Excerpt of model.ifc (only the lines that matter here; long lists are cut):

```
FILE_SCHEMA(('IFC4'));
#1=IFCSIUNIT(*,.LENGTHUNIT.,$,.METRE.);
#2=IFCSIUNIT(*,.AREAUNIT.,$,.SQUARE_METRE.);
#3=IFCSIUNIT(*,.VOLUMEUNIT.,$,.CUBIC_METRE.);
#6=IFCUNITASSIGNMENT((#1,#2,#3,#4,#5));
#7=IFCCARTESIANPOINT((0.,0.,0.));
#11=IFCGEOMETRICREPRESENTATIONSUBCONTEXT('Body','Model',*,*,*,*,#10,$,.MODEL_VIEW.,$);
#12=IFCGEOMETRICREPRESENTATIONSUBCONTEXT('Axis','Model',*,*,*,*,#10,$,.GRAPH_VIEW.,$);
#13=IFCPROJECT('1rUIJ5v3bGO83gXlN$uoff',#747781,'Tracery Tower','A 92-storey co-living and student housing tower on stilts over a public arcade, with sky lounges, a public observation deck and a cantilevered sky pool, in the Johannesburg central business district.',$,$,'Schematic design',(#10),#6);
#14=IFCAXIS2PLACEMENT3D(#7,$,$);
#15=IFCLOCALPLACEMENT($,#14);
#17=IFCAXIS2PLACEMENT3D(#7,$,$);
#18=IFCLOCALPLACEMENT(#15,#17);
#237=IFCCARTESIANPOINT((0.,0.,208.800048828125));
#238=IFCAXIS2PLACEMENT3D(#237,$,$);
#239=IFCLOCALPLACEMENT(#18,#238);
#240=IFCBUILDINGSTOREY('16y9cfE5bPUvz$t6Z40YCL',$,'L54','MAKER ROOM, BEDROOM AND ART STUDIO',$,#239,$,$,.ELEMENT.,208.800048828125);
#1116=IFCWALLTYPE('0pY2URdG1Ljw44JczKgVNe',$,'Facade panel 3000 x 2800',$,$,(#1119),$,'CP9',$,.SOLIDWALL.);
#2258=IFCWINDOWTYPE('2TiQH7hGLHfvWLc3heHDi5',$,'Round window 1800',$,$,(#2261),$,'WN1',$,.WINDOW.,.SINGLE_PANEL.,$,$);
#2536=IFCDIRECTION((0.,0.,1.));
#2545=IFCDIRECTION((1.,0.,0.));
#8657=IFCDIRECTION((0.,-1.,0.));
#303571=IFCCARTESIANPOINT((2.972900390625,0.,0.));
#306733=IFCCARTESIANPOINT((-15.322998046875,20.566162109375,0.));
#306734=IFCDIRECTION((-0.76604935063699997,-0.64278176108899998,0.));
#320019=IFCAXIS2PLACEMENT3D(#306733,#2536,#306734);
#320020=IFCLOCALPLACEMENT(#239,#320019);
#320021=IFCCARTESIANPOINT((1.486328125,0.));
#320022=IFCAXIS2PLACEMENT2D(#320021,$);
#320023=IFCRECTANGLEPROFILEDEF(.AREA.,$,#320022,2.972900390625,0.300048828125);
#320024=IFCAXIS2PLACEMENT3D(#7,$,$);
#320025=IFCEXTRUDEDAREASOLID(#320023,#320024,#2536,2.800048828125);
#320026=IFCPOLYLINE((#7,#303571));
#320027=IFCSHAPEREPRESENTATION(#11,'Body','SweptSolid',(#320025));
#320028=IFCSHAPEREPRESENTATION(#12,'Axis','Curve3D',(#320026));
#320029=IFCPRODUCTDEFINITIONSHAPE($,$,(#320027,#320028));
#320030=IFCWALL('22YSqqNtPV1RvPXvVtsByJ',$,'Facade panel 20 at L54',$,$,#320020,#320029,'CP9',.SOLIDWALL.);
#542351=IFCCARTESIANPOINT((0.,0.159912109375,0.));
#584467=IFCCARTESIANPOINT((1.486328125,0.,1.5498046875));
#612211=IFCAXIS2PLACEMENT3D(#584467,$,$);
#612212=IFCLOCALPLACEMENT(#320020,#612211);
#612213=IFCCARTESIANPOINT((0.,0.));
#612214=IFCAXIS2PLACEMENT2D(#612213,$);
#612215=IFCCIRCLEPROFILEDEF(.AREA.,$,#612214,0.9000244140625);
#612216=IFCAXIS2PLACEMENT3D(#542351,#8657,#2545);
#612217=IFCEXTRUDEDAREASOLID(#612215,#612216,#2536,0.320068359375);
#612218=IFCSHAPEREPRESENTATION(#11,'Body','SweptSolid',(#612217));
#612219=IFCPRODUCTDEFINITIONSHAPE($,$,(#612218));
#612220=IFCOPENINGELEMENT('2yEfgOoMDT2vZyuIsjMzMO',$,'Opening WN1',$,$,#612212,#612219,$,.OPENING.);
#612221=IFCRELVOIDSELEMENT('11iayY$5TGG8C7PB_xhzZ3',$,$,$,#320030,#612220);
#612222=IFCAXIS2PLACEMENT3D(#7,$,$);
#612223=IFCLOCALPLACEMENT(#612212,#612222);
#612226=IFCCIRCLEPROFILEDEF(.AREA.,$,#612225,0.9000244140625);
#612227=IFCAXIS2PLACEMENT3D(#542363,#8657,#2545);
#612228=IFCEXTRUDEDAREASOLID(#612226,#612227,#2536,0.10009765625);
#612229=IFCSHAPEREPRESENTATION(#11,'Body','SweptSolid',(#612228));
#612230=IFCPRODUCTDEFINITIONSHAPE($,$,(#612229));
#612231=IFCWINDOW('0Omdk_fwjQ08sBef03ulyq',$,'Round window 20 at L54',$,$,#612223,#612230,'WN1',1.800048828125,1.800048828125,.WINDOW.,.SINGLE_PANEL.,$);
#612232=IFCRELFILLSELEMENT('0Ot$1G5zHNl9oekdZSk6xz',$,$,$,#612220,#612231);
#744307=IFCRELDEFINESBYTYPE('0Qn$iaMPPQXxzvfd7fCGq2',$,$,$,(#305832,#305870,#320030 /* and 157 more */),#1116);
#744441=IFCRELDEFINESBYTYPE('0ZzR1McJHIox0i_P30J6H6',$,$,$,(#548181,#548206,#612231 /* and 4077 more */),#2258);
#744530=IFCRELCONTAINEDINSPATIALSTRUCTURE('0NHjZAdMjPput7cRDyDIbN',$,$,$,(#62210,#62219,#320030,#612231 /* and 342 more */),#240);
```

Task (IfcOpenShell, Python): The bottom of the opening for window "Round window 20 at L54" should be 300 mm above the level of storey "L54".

```python
import numpy as np
import ifcopenshell
import ifcopenshell.api.geometry
import ifcopenshell.geom
import ifcopenshell.util.element
import ifcopenshell.util.placement
import ifcopenshell.util.shape
import ifcopenshell.util.unit

model = ifcopenshell.open("model.ifc")
unit_scale = ifcopenshell.util.unit.calculate_unit_scale(model)

window = model.by_id(612231)
opening = window.FillsVoids[0].RelatingOpeningElement
storey = ifcopenshell.util.element.get_container(window, ifc_class="IfcBuildingStorey")
level = ifcopenshell.util.placement.get_local_placement(storey.ObjectPlacement)[2, 3]

# The opening's origin need not be at the sill, so measure its lowest point.
shape = ifcopenshell.geom.create_shape(ifcopenshell.geom.settings(), opening)
bottom = ifcopenshell.util.shape.get_shape_bottom_elevation(shape, shape.geometry) / unit_scale
dz = level + 0.3 / unit_scale - bottom

shift = np.array([0.0, 0.0, dz])
# The window is placed relative to its opening, so it follows when the opening moves.
matrix = ifcopenshell.util.placement.get_local_placement(opening.ObjectPlacement)
matrix[:3, 3] += shift
ifcopenshell.api.geometry.edit_object_placement(
    model, product=opening, matrix=matrix, is_si=False, should_transform_children=True
)

print(f"moved by {dz * unit_scale:+.3f} m")

model.write("model_updated.ifc")
```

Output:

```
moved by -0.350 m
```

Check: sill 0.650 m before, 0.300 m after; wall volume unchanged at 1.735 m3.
